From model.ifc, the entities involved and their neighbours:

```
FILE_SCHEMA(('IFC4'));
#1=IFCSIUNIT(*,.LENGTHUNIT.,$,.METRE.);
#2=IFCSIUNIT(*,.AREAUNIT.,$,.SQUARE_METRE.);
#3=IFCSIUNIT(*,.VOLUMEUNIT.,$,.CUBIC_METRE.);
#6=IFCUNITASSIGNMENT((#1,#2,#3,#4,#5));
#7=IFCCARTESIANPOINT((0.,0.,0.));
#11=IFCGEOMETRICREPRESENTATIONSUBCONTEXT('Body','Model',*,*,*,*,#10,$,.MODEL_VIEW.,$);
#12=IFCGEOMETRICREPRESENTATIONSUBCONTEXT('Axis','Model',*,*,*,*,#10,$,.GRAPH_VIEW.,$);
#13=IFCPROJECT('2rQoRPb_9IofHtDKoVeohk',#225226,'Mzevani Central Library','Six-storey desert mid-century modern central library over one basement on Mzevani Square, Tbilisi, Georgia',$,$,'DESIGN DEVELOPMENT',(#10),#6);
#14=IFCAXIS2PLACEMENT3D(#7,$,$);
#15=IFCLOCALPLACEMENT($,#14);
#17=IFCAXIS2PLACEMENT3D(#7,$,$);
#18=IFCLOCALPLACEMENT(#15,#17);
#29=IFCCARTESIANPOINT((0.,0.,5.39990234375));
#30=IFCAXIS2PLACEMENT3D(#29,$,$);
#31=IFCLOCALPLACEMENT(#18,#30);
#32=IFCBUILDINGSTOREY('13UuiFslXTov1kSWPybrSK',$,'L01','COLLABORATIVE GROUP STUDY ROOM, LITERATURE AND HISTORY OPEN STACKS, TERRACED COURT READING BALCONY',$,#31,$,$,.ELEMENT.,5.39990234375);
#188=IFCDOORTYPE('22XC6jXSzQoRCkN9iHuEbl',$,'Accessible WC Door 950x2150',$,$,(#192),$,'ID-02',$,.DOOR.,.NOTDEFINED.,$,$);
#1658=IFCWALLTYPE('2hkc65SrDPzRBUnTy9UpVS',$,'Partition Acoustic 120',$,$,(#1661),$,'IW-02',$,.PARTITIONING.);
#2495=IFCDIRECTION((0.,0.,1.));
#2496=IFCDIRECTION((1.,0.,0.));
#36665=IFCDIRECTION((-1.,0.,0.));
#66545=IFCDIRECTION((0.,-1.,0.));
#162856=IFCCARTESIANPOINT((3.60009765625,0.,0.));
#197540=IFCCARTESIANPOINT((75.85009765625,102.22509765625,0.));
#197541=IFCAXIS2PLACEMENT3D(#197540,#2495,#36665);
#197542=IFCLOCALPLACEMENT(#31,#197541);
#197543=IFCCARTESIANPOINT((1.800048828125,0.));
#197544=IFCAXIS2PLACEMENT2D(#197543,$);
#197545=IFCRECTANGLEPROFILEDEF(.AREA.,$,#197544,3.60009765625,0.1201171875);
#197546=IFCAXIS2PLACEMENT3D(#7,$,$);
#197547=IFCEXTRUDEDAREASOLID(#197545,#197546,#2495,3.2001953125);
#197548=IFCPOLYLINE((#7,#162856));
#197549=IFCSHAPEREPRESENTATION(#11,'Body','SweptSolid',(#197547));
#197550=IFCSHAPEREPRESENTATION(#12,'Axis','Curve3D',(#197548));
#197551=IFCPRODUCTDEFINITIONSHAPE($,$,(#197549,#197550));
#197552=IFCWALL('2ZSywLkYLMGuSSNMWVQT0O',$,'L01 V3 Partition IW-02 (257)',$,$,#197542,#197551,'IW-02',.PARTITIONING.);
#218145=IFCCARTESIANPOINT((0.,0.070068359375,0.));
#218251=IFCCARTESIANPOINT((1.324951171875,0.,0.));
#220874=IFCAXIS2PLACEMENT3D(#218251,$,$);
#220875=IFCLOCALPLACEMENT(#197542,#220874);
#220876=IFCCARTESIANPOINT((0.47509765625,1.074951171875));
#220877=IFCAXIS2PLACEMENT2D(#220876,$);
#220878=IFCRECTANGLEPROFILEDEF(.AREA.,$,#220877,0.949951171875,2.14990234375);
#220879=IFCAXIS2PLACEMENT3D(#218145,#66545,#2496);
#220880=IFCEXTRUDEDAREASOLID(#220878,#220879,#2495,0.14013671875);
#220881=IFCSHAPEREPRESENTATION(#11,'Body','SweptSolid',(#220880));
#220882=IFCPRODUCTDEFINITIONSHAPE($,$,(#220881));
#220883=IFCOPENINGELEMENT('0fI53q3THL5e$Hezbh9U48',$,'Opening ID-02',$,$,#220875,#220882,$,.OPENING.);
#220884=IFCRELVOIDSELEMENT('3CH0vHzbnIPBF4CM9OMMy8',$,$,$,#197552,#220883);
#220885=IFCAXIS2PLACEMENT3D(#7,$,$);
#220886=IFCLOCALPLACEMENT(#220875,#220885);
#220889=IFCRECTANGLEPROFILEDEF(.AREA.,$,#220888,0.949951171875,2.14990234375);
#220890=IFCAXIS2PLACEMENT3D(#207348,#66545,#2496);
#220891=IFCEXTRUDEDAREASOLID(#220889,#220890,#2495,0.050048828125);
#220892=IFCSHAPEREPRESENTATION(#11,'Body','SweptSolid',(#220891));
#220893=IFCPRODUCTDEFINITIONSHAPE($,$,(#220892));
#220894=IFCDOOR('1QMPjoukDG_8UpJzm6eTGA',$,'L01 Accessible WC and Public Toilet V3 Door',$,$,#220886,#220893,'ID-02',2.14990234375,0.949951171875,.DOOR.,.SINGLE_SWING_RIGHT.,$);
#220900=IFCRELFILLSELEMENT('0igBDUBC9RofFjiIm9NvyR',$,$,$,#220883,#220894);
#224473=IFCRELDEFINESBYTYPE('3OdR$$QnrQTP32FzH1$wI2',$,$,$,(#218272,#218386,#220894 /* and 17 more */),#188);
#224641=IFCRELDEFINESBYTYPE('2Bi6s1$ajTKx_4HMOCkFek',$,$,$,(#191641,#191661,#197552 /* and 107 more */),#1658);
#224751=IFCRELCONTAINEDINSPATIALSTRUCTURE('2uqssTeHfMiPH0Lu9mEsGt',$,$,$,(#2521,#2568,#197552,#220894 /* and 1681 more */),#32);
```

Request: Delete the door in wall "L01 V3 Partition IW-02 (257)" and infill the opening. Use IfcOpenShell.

```python
import ifcopenshell
import ifcopenshell.api.feature
import ifcopenshell.api.root
import ifcopenshell.geom
import ifcopenshell.util.shape

model = ifcopenshell.open("model.ifc")
settings = ifcopenshell.geom.settings()


def volume(element):
    """Net volume in cubic metres, openings subtracted."""
    shape = ifcopenshell.geom.create_shape(settings, element)
    return ifcopenshell.util.shape.get_volume(shape.geometry)


door = model.by_id(220894)
opening = door.FillsVoids[0].RelatingOpeningElement
wall = opening.VoidsElements[0].RelatingBuildingElement
before = volume(wall)

ifcopenshell.api.root.remove_product(model, product=door)
ifcopenshell.api.feature.remove_feature(model, feature=opening)

after = volume(wall)

print(f"wall volume {before:.3f} -> {after:.3f} m3")

model.write("model_v2.ifc")
```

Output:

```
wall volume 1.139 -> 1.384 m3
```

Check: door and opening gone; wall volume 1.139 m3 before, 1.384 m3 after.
